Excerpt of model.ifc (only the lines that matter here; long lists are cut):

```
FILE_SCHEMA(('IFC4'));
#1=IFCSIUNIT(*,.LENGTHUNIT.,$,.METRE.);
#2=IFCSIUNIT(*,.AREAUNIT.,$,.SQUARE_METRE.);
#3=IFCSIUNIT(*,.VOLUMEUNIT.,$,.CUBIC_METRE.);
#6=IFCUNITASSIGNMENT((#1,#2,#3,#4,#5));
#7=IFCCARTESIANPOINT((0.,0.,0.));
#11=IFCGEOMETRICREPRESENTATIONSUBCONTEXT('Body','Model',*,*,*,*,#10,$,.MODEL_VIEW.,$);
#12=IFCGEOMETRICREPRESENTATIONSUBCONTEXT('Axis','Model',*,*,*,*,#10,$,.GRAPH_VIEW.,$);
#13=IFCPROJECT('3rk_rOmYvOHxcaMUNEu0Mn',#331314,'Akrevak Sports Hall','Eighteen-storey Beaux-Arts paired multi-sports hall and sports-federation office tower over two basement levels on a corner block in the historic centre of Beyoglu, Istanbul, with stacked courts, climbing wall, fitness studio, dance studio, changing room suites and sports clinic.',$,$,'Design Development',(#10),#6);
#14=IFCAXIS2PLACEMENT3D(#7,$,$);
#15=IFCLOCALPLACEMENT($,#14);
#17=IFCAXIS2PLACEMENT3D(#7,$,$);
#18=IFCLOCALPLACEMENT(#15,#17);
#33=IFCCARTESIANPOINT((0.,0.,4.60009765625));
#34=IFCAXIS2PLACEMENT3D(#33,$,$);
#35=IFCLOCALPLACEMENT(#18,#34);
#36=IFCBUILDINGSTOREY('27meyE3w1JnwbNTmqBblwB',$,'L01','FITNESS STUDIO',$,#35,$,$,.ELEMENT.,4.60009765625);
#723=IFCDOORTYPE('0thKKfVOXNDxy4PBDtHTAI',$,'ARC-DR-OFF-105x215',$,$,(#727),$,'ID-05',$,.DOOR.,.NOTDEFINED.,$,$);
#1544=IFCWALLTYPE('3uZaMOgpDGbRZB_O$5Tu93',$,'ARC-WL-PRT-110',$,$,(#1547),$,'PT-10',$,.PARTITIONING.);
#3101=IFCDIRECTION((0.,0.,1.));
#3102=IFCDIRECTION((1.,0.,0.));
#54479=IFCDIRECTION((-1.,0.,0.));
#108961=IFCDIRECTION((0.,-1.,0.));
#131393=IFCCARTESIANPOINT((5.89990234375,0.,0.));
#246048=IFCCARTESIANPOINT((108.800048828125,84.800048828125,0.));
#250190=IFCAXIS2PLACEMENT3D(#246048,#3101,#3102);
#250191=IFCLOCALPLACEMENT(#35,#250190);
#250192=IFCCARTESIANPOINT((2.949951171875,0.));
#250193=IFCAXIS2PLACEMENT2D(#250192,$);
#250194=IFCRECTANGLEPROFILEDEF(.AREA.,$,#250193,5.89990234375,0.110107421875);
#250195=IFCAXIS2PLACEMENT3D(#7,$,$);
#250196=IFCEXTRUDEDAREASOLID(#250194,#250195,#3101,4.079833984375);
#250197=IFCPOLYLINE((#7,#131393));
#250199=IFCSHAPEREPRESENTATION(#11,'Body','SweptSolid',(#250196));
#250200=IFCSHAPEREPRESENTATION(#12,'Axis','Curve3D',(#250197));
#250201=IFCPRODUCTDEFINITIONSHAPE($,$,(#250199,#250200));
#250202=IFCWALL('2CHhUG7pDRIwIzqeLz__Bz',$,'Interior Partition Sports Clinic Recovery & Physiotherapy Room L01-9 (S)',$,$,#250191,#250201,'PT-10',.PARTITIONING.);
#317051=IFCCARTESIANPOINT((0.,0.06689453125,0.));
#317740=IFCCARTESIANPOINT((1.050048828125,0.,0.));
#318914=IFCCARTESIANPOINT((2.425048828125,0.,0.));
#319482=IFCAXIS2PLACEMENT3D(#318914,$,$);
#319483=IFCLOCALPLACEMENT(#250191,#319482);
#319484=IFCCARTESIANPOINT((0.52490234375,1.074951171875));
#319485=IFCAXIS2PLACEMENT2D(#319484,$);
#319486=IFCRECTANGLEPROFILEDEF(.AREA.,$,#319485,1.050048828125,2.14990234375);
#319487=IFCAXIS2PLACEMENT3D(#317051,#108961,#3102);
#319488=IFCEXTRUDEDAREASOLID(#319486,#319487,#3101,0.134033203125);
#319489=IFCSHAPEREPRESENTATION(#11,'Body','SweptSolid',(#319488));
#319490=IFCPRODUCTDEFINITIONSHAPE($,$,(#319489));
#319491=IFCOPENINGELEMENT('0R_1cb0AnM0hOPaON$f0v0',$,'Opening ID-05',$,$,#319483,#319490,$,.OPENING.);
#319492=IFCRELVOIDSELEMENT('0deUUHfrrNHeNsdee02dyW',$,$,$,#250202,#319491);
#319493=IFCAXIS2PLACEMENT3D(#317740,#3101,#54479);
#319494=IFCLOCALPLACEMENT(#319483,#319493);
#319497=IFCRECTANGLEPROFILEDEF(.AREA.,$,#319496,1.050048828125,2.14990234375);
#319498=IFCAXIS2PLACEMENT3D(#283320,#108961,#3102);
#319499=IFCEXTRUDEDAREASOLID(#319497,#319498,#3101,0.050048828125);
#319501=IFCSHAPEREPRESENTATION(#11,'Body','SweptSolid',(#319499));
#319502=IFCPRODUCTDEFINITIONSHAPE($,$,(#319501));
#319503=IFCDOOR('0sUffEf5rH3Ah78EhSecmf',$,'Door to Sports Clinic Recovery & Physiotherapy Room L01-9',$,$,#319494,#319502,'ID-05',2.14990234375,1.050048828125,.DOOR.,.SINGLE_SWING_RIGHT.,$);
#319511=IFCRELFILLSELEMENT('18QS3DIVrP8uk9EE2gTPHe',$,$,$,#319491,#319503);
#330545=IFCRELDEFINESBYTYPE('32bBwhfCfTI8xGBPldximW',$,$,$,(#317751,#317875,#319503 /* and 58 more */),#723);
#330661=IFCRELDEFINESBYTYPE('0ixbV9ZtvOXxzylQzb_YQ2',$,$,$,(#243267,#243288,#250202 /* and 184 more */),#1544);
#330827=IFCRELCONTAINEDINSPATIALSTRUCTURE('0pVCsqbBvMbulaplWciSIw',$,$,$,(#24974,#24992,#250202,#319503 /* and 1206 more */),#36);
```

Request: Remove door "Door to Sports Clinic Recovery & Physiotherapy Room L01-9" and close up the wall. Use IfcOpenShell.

```python
import ifcopenshell
import ifcopenshell.api.feature
import ifcopenshell.api.root
import ifcopenshell.geom
import ifcopenshell.util.shape

model = ifcopenshell.open("model.ifc")
settings = ifcopenshell.geom.settings()


def volume(element):
    """Net volume in cubic metres, openings subtracted."""
    shape = ifcopenshell.geom.create_shape(settings, element)
    return ifcopenshell.util.shape.get_volume(shape.geometry)


door = model.by_id(319503)
opening = door.FillsVoids[0].RelatingOpeningElement
wall = opening.VoidsElements[0].RelatingBuildingElement
before = volume(wall)

ifcopenshell.api.root.remove_product(model, product=door)
ifcopenshell.api.feature.remove_feature(model, feature=opening)

after = volume(wall)

print(f"wall volume {before:.3f} -> {after:.3f} m3")

model.write("model_edited.ifc")
```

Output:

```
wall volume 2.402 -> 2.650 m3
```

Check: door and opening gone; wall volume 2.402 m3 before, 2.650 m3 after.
